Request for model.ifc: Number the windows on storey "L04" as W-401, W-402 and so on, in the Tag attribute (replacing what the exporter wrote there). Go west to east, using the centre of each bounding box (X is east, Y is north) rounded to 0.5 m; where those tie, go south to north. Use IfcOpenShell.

First a look at what the model holds.

```python
import ifcopenshell
import ifcopenshell.util.element
import ifcopenshell.util.placement

model = ifcopenshell.open("model.ifc")
print(model.schema)
storey = next(s for s in model.by_type("IfcBuildingStorey") if s.Name == "L04")
windows = [e for e in ifcopenshell.util.element.get_decomposition(storey) if e.is_a("IfcWindow")]
for e in sorted(windows, key=lambda e: e.id()):
    origin = ifcopenshell.util.placement.get_local_placement(e.ObjectPlacement)[:3, 3]
    print(e.id(), e.Tag, e.Name, origin.round(2) + 0.0, sep=" | ")
```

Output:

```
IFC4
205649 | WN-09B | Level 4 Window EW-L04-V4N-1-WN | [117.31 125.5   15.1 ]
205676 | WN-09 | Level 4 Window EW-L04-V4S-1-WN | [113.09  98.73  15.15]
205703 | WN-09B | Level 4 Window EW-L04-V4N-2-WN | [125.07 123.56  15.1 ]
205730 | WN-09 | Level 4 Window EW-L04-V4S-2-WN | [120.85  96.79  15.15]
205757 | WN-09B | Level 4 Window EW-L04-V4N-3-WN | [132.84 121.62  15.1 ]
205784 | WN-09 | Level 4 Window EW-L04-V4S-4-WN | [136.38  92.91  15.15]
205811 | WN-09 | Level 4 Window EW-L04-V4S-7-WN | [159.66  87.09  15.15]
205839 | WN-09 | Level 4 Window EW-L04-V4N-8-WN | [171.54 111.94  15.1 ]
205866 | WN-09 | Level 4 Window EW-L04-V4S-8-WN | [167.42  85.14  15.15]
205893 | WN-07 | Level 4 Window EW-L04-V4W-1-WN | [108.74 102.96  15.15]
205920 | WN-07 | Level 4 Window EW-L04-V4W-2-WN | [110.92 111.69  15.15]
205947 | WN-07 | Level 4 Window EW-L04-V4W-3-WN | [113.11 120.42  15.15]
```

```python
import ifcopenshell
import ifcopenshell.geom
import ifcopenshell.util.element
import ifcopenshell.util.shape

model = ifcopenshell.open("model.ifc")
settings = ifcopenshell.geom.settings()
settings.set("use-world-coords", True)


def centre(element):
    shape = ifcopenshell.geom.create_shape(settings, element)
    return ifcopenshell.util.shape.get_bbox_centroid(shape.geometry)


storey = next(s for s in model.by_type("IfcBuildingStorey") if s.Name == "L04")
windows = [e for e in ifcopenshell.util.element.get_decomposition(storey) if e.is_a("IfcWindow")]

# Insertion points can sit at a corner or the storey origin, so sort by the geometry (in metres).
centres = {e: centre(e) for e in windows}
windows.sort(key=lambda e: (round(centres[e][0] / 0.5), centres[e][1]))

for i, e in enumerate(windows, start=1):
    number = f"W-4{i:02d}"
    e.Tag = number
    print(e.id(), number)

model.write("model-out.ifc")
```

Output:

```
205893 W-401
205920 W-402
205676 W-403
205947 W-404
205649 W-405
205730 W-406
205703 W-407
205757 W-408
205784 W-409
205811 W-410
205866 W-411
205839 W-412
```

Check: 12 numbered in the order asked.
